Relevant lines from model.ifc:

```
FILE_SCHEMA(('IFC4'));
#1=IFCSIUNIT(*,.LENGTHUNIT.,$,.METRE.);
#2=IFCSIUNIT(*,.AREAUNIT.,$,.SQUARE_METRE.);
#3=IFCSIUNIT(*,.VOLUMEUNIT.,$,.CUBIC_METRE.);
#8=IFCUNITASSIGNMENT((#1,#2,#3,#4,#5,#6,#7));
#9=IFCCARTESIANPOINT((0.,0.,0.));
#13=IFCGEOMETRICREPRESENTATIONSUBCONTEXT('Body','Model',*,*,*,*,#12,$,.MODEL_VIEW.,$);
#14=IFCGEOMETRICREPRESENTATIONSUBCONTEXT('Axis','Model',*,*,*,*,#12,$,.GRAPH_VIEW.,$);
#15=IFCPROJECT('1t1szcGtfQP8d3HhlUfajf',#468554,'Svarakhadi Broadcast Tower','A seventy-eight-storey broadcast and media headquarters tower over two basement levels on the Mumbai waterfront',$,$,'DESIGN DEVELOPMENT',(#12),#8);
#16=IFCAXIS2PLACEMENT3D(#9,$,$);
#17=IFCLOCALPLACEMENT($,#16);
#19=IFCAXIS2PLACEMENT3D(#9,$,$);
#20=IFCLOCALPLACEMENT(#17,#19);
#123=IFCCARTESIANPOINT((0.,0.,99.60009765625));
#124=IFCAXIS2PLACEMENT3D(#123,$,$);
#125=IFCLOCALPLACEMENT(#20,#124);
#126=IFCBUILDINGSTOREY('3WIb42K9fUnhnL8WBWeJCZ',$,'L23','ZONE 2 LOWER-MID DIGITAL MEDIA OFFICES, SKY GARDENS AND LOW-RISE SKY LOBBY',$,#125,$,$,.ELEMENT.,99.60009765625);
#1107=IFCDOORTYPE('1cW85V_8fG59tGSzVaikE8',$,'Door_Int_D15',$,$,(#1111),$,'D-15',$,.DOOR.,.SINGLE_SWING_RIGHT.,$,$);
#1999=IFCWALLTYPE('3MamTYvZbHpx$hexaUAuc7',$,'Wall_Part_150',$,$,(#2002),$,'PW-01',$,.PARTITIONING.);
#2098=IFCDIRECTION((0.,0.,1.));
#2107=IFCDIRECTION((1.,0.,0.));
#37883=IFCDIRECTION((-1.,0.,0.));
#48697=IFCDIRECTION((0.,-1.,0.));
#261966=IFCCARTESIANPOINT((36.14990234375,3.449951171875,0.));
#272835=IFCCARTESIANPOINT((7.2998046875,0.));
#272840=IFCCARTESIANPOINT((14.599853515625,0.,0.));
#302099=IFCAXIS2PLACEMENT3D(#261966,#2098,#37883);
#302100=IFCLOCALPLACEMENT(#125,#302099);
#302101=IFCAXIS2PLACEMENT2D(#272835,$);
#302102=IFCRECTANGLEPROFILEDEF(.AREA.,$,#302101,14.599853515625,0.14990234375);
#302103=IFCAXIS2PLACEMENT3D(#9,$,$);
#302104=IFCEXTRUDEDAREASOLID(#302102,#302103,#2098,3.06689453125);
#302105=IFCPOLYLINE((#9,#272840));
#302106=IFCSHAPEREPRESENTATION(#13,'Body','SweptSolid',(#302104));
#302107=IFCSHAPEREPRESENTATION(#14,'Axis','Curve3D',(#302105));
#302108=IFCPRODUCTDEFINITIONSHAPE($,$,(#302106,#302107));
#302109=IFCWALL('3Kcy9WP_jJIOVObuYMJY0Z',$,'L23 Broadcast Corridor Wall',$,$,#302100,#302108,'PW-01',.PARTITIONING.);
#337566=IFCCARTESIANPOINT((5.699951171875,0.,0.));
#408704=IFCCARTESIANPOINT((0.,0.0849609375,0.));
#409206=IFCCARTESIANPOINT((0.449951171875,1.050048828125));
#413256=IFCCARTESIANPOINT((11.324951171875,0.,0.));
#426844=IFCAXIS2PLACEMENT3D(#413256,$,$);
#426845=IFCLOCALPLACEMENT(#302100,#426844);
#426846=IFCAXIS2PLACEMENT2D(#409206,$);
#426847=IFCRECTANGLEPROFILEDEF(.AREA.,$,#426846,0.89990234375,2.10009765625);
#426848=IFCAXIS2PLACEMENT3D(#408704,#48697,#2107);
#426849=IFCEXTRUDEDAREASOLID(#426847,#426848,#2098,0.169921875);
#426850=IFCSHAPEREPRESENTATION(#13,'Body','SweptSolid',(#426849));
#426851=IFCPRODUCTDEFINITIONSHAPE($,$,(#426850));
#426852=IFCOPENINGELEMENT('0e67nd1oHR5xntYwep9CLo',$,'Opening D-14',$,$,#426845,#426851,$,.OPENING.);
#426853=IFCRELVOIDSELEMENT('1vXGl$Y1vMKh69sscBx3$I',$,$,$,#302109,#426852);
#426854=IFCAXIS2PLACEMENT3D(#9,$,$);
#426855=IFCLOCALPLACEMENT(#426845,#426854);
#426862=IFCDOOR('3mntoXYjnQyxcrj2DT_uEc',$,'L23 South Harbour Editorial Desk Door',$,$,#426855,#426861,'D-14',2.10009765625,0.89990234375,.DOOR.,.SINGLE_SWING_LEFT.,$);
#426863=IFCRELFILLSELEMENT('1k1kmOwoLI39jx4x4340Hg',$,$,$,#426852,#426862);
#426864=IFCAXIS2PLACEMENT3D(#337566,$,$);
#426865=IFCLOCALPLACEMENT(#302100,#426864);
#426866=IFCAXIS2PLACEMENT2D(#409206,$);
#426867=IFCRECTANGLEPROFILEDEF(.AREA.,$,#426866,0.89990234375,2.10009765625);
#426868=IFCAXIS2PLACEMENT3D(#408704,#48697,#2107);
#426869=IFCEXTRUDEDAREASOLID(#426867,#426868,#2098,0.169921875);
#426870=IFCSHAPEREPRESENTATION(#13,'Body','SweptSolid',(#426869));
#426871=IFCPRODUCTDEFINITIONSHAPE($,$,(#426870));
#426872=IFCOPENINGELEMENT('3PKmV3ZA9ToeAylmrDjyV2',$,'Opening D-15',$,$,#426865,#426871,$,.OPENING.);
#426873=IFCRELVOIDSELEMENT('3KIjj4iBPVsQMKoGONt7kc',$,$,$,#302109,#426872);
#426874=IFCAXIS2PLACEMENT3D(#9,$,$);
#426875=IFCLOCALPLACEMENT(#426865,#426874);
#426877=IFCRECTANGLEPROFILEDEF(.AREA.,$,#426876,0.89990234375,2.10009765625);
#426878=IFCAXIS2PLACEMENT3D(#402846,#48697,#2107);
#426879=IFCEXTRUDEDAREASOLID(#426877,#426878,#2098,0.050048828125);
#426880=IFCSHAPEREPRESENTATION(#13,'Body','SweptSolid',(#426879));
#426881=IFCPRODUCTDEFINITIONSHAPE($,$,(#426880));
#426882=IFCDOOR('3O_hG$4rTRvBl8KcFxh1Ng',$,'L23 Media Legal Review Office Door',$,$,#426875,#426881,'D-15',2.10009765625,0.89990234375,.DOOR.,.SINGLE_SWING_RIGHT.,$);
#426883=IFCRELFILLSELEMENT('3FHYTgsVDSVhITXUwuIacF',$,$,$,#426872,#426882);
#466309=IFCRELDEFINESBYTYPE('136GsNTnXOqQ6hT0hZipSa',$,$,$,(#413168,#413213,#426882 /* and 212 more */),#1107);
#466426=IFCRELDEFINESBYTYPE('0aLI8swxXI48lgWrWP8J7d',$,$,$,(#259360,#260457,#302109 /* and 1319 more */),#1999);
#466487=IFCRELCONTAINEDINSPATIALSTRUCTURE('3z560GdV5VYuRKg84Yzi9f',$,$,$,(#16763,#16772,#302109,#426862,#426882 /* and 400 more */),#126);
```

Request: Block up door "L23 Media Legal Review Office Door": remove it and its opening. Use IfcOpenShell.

```python
import ifcopenshell
import ifcopenshell.api.feature
import ifcopenshell.api.root
import ifcopenshell.geom
import ifcopenshell.util.shape

model = ifcopenshell.open("model.ifc")
settings = ifcopenshell.geom.settings()


def volume(element):
    """Net volume in cubic metres, openings subtracted."""
    shape = ifcopenshell.geom.create_shape(settings, element)
    return ifcopenshell.util.shape.get_volume(shape.geometry)


door = model.by_guid("3O_hG$4rTRvBl8KcFxh1Ng")
opening = door.FillsVoids[0].RelatingOpeningElement
wall = opening.VoidsElements[0].RelatingBuildingElement
before = volume(wall)

ifcopenshell.api.root.remove_product(model, product=door)
ifcopenshell.api.feature.remove_feature(model, feature=opening)

after = volume(wall)

print(f"wall volume {before:.3f} -> {after:.3f} m3")

model.write("model-out.ifc")
```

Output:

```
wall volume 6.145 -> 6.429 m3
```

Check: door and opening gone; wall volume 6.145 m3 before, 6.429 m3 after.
